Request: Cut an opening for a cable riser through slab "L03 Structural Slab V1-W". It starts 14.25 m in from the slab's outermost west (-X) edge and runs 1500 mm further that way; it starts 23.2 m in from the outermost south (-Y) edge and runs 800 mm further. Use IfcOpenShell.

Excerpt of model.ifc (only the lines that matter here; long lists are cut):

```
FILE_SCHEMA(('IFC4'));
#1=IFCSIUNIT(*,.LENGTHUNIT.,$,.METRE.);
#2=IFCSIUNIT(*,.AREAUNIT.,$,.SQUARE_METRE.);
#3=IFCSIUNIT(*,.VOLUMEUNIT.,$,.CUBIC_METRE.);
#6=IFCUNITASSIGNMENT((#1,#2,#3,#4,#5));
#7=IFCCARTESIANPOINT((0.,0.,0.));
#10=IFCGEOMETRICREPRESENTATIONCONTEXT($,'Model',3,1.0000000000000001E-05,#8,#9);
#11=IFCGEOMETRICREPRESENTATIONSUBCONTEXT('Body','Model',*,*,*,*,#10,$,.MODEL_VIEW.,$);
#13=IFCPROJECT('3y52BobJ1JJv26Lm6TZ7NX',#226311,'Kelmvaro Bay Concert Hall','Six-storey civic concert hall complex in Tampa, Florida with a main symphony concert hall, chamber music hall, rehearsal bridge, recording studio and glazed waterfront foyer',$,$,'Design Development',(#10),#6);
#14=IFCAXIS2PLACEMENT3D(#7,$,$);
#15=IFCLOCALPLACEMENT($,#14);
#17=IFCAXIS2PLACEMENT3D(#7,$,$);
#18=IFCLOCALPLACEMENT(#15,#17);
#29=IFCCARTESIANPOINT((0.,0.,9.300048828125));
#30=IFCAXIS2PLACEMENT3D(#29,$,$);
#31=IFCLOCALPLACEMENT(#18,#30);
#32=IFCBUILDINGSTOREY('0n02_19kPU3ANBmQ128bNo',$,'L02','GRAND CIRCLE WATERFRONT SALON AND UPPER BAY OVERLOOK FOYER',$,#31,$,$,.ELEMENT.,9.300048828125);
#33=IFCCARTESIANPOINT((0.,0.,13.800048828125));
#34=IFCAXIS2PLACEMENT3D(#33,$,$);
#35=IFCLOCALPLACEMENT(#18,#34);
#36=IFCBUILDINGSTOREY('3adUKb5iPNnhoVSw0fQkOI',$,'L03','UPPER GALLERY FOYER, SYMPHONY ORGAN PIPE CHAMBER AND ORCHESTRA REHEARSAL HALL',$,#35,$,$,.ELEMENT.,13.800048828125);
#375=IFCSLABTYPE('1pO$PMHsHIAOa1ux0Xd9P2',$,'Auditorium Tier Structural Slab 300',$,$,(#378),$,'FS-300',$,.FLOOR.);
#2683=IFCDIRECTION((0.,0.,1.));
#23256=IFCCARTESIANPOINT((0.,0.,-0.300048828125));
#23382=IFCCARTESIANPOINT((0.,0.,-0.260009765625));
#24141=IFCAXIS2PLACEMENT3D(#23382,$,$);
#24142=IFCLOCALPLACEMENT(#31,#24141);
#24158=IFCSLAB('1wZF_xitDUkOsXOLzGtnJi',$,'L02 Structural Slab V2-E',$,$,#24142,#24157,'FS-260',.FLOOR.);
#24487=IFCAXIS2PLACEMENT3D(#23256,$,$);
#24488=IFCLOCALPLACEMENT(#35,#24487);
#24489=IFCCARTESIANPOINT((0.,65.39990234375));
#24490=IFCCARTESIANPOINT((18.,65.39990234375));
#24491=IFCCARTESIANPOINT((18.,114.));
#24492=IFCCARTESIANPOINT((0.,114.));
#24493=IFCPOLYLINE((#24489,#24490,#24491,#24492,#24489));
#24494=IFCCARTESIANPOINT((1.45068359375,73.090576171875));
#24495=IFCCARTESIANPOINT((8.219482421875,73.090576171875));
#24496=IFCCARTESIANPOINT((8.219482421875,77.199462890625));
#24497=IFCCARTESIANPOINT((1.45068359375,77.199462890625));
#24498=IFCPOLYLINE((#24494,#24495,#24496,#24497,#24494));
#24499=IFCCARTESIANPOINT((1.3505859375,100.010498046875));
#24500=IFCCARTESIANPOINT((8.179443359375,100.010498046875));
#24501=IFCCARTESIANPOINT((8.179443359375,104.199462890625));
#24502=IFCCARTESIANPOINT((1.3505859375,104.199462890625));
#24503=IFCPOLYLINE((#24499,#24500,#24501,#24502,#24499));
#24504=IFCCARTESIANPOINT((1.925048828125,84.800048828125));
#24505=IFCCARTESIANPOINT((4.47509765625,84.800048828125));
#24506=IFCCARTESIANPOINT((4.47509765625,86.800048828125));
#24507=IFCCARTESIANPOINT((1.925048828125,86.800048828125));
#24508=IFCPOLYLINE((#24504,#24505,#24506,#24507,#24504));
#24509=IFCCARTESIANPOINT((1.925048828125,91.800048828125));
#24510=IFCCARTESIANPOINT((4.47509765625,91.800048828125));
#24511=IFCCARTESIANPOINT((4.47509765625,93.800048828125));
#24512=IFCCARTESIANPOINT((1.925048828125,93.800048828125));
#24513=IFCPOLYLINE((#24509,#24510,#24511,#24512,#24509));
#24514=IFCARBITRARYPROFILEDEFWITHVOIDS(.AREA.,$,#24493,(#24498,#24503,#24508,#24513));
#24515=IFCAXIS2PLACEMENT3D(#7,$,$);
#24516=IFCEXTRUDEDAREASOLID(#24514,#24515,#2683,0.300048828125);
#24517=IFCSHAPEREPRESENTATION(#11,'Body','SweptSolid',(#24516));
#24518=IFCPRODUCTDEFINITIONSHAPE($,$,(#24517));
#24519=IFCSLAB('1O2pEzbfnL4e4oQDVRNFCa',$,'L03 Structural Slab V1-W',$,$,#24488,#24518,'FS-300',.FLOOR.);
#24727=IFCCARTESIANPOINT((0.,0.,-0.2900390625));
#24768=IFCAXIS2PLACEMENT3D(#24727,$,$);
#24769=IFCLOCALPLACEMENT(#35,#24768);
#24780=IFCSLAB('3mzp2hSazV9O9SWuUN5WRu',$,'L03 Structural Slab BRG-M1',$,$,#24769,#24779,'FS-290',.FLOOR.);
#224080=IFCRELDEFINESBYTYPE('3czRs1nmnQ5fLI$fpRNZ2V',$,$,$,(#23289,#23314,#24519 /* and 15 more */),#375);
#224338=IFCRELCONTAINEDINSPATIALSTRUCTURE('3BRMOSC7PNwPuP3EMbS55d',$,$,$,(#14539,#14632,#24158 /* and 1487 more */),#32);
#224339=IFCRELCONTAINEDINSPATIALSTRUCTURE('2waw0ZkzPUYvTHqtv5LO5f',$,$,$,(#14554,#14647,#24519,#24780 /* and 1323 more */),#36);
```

```python
import numpy as np
import ifcopenshell
import ifcopenshell.api.feature
import ifcopenshell.api.geometry
import ifcopenshell.api.root
import ifcopenshell.geom
import ifcopenshell.util.placement
import ifcopenshell.util.representation
import ifcopenshell.util.shape
import ifcopenshell.util.unit

model = ifcopenshell.open("model.ifc")
unit_scale = ifcopenshell.util.unit.calculate_unit_scale(model)
settings = ifcopenshell.geom.settings()


def volume(element):
    """Net volume in cubic metres, openings subtracted."""
    shape = ifcopenshell.geom.create_shape(settings, element)
    return ifcopenshell.util.shape.get_volume(shape.geometry)


slab = model.by_guid("1O2pEzbfnL4e4oQDVRNFCa")
before = volume(slab)

# Extent in the slab's own axes, in metres. The edges named are its -X and -Y sides.
slab_shape = ifcopenshell.geom.create_shape(settings, slab)
vertices = ifcopenshell.util.shape.get_vertices(slab_shape.geometry)
x_min, y_min, bottom = vertices.min(axis=0)
top = vertices[:, 2].max()

opening = ifcopenshell.api.root.create_entity(model, ifc_class="IfcOpeningElement", name="Cable riser opening", predefined_type="OPENING")
context = ifcopenshell.util.representation.get_context(model, "Model", "Body", "MODEL_VIEW")
width, depth = 1.5, 0.8
outline = [(0.0, 0.0), (width, 0.0), (width, depth), (0.0, depth), (0.0, 0.0)]
# Overshoot both faces by 50 mm so the cut is clean.
shape = ifcopenshell.api.geometry.add_slab_representation(
    model, context=context, depth=top - bottom + 0.1, polyline=outline
)
ifcopenshell.api.geometry.assign_representation(model, product=opening, representation=shape)

matrix = ifcopenshell.util.placement.get_local_placement(slab.ObjectPlacement)
matrix[:, 3] = matrix @ np.append(np.array([x_min + 14.25, y_min + 23.2, bottom - 0.05]) / unit_scale, 1.0)
ifcopenshell.api.geometry.edit_object_placement(model, product=opening, matrix=matrix, is_si=False)
ifcopenshell.api.feature.add_feature(model, feature=opening, element=slab)

after = volume(slab)

print(f"slab volume {before:.3f} -> {after:.3f} m3")

model.write("model_rev.ifc")
```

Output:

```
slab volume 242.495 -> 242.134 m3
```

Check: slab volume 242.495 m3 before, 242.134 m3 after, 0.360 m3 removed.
